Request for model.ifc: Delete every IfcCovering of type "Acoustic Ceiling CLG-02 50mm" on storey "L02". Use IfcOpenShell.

First a look at what the model holds.

```python
import ifcopenshell
import ifcopenshell.util.element

model = ifcopenshell.open("model.ifc")
print(model.schema)
storey = next(s for s in model.by_type("IfcBuildingStorey") if s.Name == "L02")
coverings = [e for e in ifcopenshell.util.element.get_decomposition(storey) if e.is_a("IfcCovering")]
seen = {}
for e in coverings:
    element_type = ifcopenshell.util.element.get_type(e)
    name = element_type.Name if element_type not in (None, e) else None
    seen[name] = seen.get(name, 0) + 1
for name, count in sorted(seen.items(), key=str):
    print(count, "x", name)
```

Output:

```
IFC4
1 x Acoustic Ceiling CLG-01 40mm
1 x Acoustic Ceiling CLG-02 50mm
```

```python
import ifcopenshell
import ifcopenshell.api.root
import ifcopenshell.util.element

model = ifcopenshell.open("model.ifc")

storey = next(s for s in model.by_type("IfcBuildingStorey") if s.Name == "L02")
coverings = [e for e in ifcopenshell.util.element.get_decomposition(storey) if e.is_a("IfcCovering")]
targets = [e for e in coverings if (t := ifcopenshell.util.element.get_type(e)) not in (None, e) and t.Name == "Acoustic Ceiling CLG-02 50mm"]

for e in targets:
    ifcopenshell.api.root.remove_product(model, product=e)
print(len(targets), "removed")

model.write("model_edited.ifc")
```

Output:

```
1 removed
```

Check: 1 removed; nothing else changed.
